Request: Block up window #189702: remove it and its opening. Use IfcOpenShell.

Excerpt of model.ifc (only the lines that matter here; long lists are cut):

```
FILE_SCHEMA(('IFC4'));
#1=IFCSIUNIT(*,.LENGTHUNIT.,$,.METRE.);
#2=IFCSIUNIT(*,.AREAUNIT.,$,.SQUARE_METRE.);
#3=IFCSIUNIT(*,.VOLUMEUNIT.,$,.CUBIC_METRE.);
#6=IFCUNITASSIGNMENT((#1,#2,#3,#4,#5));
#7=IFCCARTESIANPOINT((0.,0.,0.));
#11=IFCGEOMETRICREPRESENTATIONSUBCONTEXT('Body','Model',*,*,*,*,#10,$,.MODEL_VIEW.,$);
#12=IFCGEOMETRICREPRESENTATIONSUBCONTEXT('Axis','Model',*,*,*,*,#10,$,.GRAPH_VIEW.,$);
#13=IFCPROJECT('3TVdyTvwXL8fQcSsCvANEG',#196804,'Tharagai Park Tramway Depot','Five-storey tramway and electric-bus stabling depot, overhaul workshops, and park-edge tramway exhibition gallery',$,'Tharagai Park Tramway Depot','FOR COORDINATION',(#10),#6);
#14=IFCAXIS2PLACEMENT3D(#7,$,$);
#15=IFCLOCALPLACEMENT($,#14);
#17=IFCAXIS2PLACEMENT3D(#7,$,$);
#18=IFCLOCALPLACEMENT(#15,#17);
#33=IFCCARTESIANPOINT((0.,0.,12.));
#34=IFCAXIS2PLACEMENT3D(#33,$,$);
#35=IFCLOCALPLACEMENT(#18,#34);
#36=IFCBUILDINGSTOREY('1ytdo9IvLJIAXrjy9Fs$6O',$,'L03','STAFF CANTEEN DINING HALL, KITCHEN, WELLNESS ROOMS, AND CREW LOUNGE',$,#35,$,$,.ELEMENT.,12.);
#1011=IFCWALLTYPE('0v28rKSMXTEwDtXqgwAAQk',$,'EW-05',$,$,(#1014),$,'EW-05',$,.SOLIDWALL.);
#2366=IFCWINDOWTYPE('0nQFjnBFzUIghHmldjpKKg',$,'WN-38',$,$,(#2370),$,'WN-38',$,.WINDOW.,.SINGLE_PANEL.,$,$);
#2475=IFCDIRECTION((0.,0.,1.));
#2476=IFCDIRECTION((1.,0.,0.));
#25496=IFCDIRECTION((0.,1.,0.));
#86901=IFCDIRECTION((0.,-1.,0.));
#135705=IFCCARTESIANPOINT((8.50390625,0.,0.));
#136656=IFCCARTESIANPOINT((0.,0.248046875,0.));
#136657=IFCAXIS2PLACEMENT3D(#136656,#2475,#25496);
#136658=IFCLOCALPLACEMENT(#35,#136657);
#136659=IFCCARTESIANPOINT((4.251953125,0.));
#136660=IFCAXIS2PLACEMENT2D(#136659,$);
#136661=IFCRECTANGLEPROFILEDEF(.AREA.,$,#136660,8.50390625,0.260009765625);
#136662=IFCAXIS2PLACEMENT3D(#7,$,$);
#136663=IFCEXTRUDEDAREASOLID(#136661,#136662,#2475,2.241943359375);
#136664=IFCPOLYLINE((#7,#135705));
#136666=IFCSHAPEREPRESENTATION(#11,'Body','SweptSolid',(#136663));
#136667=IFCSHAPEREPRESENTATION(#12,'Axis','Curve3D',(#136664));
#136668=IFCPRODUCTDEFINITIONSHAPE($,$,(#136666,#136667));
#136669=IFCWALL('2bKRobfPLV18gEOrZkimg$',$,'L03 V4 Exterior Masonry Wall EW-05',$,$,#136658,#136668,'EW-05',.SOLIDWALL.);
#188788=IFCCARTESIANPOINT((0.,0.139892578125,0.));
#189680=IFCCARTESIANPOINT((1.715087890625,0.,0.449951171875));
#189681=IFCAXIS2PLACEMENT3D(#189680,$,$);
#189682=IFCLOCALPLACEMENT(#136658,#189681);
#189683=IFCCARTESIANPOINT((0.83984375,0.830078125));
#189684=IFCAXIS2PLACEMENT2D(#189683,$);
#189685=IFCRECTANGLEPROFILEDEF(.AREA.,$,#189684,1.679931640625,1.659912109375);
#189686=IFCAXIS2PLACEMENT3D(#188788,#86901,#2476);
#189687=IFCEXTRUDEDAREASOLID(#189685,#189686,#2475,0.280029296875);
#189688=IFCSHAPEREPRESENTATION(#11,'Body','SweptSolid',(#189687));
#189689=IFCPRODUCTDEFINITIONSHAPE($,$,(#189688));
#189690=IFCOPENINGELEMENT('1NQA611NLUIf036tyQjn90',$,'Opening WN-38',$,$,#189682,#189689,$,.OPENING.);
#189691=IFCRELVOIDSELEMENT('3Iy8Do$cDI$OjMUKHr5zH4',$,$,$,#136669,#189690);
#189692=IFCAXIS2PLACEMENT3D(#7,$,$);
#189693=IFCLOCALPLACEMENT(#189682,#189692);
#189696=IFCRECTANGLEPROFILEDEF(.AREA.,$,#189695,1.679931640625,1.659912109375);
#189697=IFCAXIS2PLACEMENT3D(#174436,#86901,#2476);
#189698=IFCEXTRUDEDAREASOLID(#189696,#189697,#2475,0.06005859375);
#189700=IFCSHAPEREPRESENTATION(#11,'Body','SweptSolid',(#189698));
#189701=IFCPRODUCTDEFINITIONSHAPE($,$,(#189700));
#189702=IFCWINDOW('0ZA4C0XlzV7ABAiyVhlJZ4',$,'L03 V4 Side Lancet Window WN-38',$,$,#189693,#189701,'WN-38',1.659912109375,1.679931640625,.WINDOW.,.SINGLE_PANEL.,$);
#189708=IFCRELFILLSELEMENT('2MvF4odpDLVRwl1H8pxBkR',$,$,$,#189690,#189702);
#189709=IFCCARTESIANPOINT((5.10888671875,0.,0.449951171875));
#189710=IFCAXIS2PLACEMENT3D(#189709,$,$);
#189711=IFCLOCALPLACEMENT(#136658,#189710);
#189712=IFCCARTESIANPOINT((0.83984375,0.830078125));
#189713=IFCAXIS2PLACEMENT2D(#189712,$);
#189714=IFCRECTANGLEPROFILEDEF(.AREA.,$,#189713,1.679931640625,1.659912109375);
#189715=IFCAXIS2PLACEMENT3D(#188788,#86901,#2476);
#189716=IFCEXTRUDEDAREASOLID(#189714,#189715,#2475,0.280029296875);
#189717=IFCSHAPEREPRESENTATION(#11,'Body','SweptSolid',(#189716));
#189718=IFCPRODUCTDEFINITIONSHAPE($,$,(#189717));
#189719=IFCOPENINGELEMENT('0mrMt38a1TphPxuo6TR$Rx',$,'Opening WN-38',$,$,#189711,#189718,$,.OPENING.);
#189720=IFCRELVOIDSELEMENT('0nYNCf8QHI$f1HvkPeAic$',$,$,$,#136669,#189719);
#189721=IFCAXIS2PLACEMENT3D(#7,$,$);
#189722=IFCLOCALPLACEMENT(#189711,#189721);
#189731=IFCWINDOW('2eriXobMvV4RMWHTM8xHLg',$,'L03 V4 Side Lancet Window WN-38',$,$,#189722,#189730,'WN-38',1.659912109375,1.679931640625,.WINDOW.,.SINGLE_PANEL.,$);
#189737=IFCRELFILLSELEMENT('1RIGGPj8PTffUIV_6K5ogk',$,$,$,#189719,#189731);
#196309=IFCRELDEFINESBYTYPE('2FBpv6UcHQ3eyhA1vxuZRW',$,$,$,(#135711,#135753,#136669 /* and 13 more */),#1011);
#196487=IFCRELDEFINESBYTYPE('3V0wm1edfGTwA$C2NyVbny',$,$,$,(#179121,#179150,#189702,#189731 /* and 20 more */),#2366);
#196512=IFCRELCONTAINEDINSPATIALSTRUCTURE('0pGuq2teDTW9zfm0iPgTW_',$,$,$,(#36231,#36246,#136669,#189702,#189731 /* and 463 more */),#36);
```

```python
import ifcopenshell
import ifcopenshell.api.feature
import ifcopenshell.api.root
import ifcopenshell.geom
import ifcopenshell.util.shape

model = ifcopenshell.open("model.ifc")
settings = ifcopenshell.geom.settings()


def volume(element):
    """Net volume in cubic metres, openings subtracted."""
    shape = ifcopenshell.geom.create_shape(settings, element)
    return ifcopenshell.util.shape.get_volume(shape.geometry)


window = model.by_guid("0ZA4C0XlzV7ABAiyVhlJZ4")
opening = window.FillsVoids[0].RelatingOpeningElement
wall = opening.VoidsElements[0].RelatingBuildingElement
before = volume(wall)

ifcopenshell.api.root.remove_product(model, product=window)
ifcopenshell.api.feature.remove_feature(model, feature=opening)

after = volume(wall)

print(f"wall volume {before:.3f} -> {after:.3f} m3")

model.write("model_v2.ifc")
```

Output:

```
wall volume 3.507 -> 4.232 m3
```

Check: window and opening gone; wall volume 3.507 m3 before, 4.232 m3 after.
